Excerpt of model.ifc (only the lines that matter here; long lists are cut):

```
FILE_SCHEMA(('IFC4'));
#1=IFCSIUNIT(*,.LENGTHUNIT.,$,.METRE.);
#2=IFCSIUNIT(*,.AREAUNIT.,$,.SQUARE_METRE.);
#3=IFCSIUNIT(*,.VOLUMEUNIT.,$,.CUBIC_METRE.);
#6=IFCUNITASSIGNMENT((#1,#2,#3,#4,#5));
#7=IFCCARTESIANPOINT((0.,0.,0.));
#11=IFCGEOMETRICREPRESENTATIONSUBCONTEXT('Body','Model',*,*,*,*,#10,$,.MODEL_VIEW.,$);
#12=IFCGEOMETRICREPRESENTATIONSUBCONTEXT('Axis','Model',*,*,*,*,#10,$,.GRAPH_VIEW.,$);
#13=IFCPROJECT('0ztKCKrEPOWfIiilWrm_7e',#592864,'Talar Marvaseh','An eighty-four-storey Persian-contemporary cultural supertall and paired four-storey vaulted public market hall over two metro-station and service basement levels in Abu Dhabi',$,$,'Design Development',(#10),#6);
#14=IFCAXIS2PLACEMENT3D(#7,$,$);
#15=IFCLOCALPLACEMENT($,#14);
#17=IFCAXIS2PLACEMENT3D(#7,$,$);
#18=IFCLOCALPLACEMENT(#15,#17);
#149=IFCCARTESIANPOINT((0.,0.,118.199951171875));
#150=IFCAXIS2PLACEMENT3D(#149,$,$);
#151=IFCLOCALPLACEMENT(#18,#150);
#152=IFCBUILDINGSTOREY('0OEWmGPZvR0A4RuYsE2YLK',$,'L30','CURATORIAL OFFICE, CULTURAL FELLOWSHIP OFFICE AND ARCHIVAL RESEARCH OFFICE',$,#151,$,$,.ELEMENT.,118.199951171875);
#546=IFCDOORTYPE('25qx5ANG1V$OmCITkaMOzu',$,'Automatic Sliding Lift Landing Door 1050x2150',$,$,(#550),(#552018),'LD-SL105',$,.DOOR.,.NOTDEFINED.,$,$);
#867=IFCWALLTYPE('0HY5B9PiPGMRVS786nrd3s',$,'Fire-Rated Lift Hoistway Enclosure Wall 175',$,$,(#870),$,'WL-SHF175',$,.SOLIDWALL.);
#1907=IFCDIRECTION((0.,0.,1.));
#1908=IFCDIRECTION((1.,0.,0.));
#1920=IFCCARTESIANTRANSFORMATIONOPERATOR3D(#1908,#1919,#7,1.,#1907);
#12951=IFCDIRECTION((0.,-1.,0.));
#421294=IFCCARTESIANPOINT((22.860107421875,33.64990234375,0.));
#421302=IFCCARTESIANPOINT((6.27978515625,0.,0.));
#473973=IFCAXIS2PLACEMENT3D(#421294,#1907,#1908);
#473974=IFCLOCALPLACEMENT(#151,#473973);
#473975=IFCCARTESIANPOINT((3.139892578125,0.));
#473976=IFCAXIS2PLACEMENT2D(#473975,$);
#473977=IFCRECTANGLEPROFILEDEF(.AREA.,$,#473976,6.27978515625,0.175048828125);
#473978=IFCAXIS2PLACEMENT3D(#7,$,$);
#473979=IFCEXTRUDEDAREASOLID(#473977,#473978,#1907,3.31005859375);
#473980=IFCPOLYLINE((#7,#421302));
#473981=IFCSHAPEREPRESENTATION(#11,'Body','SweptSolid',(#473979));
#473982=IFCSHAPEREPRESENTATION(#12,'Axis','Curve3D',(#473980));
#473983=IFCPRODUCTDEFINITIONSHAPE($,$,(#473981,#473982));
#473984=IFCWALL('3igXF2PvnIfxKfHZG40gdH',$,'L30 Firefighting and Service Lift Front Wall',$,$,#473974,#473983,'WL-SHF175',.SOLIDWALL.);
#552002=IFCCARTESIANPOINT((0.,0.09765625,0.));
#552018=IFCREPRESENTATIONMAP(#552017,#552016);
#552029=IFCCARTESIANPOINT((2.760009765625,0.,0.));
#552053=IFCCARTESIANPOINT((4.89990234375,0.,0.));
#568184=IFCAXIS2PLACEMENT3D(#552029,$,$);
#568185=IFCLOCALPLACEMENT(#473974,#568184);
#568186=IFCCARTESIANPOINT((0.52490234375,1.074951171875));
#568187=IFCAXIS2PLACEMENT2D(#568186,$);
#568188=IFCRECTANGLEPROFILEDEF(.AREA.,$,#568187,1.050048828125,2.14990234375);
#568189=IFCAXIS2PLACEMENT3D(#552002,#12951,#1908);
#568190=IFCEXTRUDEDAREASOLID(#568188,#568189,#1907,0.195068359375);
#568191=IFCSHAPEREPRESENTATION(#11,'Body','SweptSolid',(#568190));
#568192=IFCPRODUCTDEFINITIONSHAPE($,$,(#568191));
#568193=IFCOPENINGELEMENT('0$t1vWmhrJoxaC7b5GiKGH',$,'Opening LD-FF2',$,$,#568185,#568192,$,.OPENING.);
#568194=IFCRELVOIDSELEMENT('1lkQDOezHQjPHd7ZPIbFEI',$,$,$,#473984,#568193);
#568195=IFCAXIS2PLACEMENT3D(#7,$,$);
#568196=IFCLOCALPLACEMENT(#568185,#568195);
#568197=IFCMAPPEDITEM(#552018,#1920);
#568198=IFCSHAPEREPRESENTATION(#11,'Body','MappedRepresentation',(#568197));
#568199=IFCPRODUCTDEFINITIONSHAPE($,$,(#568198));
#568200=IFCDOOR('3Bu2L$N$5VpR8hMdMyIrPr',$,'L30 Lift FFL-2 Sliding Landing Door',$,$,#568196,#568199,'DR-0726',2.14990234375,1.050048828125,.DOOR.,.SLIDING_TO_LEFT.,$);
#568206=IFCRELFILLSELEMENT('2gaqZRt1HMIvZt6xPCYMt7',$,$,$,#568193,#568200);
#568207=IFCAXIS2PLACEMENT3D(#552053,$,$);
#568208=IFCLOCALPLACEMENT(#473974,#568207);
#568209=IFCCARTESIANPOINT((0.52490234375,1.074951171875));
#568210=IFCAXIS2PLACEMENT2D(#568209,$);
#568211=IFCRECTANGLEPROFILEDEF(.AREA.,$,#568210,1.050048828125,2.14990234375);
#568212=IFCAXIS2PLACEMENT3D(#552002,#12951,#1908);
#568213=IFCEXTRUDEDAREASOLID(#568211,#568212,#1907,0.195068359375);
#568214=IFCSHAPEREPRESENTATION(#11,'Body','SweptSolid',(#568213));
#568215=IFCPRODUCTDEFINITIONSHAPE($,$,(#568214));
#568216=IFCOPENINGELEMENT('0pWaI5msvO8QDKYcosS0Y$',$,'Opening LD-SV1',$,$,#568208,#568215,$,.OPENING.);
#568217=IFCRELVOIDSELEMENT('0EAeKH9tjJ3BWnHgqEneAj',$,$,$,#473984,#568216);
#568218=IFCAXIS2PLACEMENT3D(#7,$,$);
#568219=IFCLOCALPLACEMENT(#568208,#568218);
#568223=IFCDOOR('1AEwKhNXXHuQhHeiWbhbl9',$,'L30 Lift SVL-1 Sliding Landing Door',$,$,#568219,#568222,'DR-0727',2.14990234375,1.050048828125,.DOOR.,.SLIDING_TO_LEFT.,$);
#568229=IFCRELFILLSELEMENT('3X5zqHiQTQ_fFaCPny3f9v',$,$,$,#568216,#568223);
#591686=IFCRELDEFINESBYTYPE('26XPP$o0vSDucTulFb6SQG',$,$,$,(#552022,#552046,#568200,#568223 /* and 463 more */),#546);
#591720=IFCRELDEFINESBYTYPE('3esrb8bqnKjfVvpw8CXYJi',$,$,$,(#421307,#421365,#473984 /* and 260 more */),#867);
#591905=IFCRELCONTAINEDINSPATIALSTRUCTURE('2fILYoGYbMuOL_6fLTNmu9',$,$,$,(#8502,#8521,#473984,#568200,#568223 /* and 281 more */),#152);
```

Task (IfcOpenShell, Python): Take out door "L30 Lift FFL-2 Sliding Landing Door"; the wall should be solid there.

```python
import ifcopenshell
import ifcopenshell.api.feature
import ifcopenshell.api.root
import ifcopenshell.geom
import ifcopenshell.util.shape

model = ifcopenshell.open("model.ifc")
settings = ifcopenshell.geom.settings()


def volume(element):
    """Net volume in cubic metres, openings subtracted."""
    shape = ifcopenshell.geom.create_shape(settings, element)
    return ifcopenshell.util.shape.get_volume(shape.geometry)


door = model.by_guid("3Bu2L$N$5VpR8hMdMyIrPr")
opening = door.FillsVoids[0].RelatingOpeningElement
wall = opening.VoidsElements[0].RelatingBuildingElement
before = volume(wall)

ifcopenshell.api.root.remove_product(model, product=door)
ifcopenshell.api.feature.remove_feature(model, feature=opening)

after = volume(wall)

print(f"wall volume {before:.3f} -> {after:.3f} m3")

model.write("model_rev.ifc")
```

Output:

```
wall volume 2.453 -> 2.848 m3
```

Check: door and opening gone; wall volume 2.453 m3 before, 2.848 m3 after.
